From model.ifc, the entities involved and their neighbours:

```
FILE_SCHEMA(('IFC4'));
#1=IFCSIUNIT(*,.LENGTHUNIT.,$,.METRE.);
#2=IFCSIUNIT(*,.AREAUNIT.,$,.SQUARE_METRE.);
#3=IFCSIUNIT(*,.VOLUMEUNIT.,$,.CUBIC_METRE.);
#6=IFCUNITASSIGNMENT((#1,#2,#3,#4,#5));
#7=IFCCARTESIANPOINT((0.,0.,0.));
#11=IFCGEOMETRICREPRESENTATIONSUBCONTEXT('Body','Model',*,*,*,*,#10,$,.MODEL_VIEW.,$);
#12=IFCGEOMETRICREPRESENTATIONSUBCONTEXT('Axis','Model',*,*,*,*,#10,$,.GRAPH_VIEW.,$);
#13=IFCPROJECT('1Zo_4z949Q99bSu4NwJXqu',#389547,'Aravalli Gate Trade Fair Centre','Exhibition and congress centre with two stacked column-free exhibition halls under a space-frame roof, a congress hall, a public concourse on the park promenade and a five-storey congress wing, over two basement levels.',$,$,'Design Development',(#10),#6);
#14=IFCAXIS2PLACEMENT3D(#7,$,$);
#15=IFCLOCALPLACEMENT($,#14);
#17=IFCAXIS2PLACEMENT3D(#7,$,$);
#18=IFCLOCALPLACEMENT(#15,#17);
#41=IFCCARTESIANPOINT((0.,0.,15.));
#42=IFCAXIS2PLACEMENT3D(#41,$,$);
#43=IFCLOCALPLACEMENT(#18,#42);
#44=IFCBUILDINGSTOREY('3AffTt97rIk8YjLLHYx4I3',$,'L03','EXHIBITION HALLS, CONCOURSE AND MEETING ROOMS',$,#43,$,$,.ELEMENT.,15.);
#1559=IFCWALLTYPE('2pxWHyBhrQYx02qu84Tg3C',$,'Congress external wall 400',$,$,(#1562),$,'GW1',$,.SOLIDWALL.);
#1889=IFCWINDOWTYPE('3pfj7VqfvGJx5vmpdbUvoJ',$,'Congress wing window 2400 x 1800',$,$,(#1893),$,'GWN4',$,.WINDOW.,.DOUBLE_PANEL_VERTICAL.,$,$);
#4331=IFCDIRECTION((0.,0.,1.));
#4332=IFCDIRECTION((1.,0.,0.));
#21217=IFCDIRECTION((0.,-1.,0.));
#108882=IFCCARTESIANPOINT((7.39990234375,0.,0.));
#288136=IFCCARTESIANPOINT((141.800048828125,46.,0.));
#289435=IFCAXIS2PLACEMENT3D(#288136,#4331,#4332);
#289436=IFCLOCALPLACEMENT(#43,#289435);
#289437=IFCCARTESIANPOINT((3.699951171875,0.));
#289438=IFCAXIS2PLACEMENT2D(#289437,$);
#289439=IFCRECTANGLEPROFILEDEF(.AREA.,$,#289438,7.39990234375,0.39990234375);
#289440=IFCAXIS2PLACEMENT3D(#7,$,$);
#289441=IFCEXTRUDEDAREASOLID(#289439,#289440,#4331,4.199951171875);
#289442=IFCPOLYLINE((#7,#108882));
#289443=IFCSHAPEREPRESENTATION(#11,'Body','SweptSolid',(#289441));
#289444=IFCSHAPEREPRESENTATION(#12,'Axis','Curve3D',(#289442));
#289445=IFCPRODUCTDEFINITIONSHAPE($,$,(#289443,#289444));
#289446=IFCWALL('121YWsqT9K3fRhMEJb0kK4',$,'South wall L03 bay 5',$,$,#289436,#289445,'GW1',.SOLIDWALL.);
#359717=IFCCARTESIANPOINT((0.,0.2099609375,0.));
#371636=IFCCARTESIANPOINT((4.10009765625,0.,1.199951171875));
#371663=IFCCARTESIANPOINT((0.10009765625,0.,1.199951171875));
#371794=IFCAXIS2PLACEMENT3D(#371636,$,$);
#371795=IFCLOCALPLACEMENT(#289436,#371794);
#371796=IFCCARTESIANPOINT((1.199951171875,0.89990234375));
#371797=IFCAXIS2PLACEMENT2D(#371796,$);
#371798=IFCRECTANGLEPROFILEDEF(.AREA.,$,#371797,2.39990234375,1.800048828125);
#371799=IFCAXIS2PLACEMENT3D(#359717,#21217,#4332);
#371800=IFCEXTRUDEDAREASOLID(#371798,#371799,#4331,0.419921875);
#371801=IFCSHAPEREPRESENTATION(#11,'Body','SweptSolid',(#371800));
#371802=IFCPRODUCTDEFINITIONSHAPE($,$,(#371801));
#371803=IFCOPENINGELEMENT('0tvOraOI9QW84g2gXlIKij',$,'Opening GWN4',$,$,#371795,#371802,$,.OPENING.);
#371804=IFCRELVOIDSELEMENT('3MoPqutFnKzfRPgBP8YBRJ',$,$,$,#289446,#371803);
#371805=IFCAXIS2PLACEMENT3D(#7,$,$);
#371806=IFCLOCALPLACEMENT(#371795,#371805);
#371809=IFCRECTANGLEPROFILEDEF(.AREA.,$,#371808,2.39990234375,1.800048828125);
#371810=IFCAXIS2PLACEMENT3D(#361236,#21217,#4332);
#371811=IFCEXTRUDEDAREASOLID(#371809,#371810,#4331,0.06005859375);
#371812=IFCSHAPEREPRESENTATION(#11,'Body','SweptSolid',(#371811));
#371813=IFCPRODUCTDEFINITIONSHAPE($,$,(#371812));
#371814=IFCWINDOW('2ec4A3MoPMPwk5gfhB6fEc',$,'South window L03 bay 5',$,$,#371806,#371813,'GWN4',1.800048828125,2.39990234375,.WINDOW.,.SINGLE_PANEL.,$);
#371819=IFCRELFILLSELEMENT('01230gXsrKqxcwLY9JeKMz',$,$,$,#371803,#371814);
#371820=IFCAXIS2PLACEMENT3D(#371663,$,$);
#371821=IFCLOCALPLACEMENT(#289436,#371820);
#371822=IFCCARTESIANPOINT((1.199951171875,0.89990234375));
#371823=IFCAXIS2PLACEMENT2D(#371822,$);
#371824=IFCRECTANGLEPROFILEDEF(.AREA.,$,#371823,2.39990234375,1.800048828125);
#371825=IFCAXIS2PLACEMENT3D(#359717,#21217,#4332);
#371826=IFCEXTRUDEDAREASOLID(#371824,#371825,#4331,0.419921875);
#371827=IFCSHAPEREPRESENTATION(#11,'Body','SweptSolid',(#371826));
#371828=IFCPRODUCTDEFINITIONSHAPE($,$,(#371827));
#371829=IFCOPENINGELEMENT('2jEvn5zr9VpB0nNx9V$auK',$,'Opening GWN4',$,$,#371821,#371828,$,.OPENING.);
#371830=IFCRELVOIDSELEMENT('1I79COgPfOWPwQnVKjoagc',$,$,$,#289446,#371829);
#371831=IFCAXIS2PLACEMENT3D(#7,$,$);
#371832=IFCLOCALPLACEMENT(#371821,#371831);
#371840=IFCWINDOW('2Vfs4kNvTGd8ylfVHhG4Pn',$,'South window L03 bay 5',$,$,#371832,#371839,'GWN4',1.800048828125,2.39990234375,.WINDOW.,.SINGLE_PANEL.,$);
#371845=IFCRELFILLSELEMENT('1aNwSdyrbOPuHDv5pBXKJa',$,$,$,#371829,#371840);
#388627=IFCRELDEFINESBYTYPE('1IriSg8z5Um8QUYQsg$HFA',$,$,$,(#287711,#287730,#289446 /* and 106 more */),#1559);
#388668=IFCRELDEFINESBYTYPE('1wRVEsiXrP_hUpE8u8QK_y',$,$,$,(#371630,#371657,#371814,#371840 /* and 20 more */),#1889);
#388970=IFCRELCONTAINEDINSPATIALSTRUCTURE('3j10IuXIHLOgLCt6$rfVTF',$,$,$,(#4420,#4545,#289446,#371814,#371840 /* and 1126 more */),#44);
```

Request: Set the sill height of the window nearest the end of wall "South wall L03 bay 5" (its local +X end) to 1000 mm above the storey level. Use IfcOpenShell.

```python
import numpy as np
import ifcopenshell
import ifcopenshell.api.geometry
import ifcopenshell.geom
import ifcopenshell.util.element
import ifcopenshell.util.placement
import ifcopenshell.util.shape
import ifcopenshell.util.unit

model = ifcopenshell.open("model.ifc")
unit_scale = ifcopenshell.util.unit.calculate_unit_scale(model)

window = model.by_guid("2ec4A3MoPMPwk5gfhB6fEc")
opening = window.FillsVoids[0].RelatingOpeningElement
storey = ifcopenshell.util.element.get_container(window, ifc_class="IfcBuildingStorey")
level = ifcopenshell.util.placement.get_local_placement(storey.ObjectPlacement)[2, 3]

# The opening's origin need not be at the sill, so measure its lowest point.
shape = ifcopenshell.geom.create_shape(ifcopenshell.geom.settings(), opening)
bottom = ifcopenshell.util.shape.get_shape_bottom_elevation(shape, shape.geometry) / unit_scale
dz = level + 1 / unit_scale - bottom

shift = np.array([0.0, 0.0, dz])
# The window is placed relative to its opening, so it follows when the opening moves.
matrix = ifcopenshell.util.placement.get_local_placement(opening.ObjectPlacement)
matrix[:3, 3] += shift
ifcopenshell.api.geometry.edit_object_placement(
    model, product=opening, matrix=matrix, is_si=False, should_transform_children=True
)

print(f"moved by {dz * unit_scale:+.3f} m")

model.write("model-out.ifc")
```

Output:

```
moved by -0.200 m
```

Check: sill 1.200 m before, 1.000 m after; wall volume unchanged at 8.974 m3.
